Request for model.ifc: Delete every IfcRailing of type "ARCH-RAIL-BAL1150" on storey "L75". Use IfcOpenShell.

First a look at what the model holds.

```python
import ifcopenshell
import ifcopenshell.util.element

model = ifcopenshell.open("model.ifc")
print(model.schema)
storey = next(s for s in model.by_type("IfcBuildingStorey") if s.Name == "L75")
railings = [e for e in ifcopenshell.util.element.get_decomposition(storey) if e.is_a("IfcRailing")]
seen = {}
for e in railings:
    element_type = ifcopenshell.util.element.get_type(e)
    name = element_type.Name if element_type not in (None, e) else None
    seen[name] = seen.get(name, 0) + 1
for name, count in sorted(seen.items(), key=str):
    print(count, "x", name)
```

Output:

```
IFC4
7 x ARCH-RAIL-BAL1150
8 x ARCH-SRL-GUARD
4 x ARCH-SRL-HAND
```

```python
import ifcopenshell
import ifcopenshell.api.root
import ifcopenshell.util.element

model = ifcopenshell.open("model.ifc")

storey = next(s for s in model.by_type("IfcBuildingStorey") if s.Name == "L75")
railings = [e for e in ifcopenshell.util.element.get_decomposition(storey) if e.is_a("IfcRailing")]
targets = [e for e in railings if (t := ifcopenshell.util.element.get_type(e)) not in (None, e) and t.Name == "ARCH-RAIL-BAL1150"]

for e in targets:
    ifcopenshell.api.root.remove_product(model, product=e)
print(len(targets), "removed")

model.write("model_edited.ifc")
```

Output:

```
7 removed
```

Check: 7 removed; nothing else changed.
